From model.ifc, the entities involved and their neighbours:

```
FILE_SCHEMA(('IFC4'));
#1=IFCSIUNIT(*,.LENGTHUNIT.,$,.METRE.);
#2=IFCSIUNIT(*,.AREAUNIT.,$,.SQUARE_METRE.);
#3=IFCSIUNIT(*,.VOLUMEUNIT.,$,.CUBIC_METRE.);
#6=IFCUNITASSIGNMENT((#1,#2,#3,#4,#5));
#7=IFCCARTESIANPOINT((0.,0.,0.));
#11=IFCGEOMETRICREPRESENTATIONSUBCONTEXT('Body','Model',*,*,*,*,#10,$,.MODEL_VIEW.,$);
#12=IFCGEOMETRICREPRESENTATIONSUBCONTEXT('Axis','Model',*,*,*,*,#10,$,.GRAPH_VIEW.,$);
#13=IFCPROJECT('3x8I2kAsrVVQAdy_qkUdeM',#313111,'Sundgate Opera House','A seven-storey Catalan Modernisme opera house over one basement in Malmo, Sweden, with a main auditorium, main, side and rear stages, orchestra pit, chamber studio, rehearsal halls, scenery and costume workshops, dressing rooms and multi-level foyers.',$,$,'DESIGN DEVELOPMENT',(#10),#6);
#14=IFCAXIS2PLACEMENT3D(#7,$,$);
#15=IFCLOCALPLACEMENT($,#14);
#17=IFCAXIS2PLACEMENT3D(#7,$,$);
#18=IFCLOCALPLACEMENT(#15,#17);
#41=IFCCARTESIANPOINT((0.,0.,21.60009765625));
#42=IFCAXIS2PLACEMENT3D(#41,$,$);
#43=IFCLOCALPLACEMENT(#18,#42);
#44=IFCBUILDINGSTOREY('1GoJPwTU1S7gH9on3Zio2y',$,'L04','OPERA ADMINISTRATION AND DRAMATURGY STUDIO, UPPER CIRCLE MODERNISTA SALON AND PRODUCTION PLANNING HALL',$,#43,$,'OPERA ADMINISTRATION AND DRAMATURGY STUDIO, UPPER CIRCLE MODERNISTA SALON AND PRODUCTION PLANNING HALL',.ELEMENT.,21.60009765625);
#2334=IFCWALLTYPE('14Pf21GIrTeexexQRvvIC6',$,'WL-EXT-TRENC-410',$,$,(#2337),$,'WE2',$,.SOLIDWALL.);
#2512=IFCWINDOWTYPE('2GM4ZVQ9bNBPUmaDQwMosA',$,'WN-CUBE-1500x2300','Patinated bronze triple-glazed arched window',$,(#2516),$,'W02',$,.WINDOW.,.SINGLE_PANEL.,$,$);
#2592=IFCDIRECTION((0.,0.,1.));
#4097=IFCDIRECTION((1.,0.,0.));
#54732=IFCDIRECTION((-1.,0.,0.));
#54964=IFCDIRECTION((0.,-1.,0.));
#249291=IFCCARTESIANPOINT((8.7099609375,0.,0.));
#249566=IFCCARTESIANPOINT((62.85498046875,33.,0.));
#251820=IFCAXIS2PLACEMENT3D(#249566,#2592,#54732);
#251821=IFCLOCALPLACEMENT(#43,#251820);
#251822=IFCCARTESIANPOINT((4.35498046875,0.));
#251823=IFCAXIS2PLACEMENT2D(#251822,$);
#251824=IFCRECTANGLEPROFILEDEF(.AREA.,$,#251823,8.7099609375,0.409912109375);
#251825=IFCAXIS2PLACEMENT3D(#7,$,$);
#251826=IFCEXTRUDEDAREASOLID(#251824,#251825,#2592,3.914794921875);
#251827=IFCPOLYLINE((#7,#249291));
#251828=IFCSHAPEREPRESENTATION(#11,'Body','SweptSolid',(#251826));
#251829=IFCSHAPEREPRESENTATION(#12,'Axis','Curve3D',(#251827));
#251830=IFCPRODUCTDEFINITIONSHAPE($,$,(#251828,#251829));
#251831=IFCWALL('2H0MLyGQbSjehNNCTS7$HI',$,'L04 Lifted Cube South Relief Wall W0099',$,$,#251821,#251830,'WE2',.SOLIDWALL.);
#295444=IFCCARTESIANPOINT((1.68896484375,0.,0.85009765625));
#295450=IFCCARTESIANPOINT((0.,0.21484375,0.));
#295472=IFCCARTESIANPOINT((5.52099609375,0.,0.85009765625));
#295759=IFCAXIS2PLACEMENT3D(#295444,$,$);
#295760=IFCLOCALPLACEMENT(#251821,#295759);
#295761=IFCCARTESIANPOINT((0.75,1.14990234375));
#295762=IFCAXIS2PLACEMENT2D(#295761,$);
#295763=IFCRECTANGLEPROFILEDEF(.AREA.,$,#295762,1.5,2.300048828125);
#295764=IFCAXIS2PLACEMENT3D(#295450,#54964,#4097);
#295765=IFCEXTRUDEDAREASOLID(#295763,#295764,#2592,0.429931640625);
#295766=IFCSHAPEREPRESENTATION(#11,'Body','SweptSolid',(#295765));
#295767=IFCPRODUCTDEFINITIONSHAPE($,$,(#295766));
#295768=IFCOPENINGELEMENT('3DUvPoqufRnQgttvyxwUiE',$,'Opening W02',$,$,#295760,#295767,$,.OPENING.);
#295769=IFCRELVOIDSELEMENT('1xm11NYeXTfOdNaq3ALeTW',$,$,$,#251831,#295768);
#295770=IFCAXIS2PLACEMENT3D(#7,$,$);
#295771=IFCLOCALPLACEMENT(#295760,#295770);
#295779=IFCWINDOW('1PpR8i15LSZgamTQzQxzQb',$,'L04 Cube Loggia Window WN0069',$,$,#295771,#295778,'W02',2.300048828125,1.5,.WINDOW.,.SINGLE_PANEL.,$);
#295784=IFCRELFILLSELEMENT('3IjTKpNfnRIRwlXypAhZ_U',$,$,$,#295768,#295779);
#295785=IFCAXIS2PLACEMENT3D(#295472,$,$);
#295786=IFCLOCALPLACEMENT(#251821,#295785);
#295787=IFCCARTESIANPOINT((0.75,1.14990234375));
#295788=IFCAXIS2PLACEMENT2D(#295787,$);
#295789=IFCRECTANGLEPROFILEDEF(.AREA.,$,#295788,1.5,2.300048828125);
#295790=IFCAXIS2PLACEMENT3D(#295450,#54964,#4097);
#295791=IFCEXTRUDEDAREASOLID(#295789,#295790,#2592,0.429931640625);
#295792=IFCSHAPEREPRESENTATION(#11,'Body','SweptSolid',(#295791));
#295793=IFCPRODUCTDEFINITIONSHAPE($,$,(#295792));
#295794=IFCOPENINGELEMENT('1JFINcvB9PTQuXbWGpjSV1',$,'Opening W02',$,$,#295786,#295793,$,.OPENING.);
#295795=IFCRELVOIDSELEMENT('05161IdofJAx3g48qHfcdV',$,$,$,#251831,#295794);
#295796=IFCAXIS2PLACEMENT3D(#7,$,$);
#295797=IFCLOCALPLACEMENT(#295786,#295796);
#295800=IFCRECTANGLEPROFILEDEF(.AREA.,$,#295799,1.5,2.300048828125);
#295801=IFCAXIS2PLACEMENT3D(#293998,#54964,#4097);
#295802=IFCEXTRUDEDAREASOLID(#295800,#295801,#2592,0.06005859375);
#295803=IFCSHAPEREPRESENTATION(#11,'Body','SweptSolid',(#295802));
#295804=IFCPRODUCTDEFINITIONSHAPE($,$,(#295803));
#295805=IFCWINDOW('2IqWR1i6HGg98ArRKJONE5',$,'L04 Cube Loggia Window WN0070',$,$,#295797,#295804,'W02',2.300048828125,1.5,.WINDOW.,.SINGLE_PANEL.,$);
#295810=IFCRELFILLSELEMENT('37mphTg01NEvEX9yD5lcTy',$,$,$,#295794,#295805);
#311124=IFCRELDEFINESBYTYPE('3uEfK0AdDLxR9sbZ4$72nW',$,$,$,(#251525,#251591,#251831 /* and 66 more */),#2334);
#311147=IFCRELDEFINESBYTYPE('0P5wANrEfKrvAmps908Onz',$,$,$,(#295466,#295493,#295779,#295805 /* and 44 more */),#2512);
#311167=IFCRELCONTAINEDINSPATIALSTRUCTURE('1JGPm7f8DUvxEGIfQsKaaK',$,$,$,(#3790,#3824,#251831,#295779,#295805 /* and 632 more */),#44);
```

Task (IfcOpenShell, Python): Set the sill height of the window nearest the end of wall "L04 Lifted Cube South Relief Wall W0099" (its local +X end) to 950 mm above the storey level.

```python
import numpy as np
import ifcopenshell
import ifcopenshell.api.geometry
import ifcopenshell.geom
import ifcopenshell.util.element
import ifcopenshell.util.placement
import ifcopenshell.util.shape
import ifcopenshell.util.unit

model = ifcopenshell.open("model.ifc")
unit_scale = ifcopenshell.util.unit.calculate_unit_scale(model)

window = model.by_id(295805)
opening = window.FillsVoids[0].RelatingOpeningElement
storey = ifcopenshell.util.element.get_container(window, ifc_class="IfcBuildingStorey")
level = ifcopenshell.util.placement.get_local_placement(storey.ObjectPlacement)[2, 3]

# The opening's origin need not be at the sill, so measure its lowest point.
shape = ifcopenshell.geom.create_shape(ifcopenshell.geom.settings(), opening)
bottom = ifcopenshell.util.shape.get_shape_bottom_elevation(shape, shape.geometry) / unit_scale
dz = level + 0.95 / unit_scale - bottom

shift = np.array([0.0, 0.0, dz])
# The window is placed relative to its opening, so it follows when the opening moves.
matrix = ifcopenshell.util.placement.get_local_placement(opening.ObjectPlacement)
matrix[:3, 3] += shift
ifcopenshell.api.geometry.edit_object_placement(
    model, product=opening, matrix=matrix, is_si=False, should_transform_children=True
)

print(f"moved by {dz * unit_scale:+.3f} m")

model.write("model_updated.ifc")
```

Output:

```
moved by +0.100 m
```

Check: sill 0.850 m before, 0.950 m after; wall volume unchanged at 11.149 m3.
